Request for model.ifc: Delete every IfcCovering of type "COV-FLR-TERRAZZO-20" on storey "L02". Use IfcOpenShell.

First a look at what the model holds.

```python
import ifcopenshell
import ifcopenshell.util.element

model = ifcopenshell.open("model.ifc")
print(model.schema)
storey = next(s for s in model.by_type("IfcBuildingStorey") if s.Name == "L02")
coverings = [e for e in ifcopenshell.util.element.get_decomposition(storey) if e.is_a("IfcCovering")]
seen = {}
for e in coverings:
    element_type = ifcopenshell.util.element.get_type(e)
    name = element_type.Name if element_type not in (None, e) else None
    seen[name] = seen.get(name, 0) + 1
for name, count in sorted(seen.items(), key=str):
    print(count, "x", name)
```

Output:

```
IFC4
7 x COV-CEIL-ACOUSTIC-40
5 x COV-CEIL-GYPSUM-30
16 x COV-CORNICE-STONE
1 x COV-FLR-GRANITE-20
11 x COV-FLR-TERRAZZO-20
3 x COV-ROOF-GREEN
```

```python
import ifcopenshell
import ifcopenshell.api.root
import ifcopenshell.util.element

model = ifcopenshell.open("model.ifc")

storey = next(s for s in model.by_type("IfcBuildingStorey") if s.Name == "L02")
coverings = [e for e in ifcopenshell.util.element.get_decomposition(storey) if e.is_a("IfcCovering")]
targets = [e for e in coverings if (t := ifcopenshell.util.element.get_type(e)) not in (None, e) and t.Name == "COV-FLR-TERRAZZO-20"]

for e in targets:
    ifcopenshell.api.root.remove_product(model, product=e)
print(len(targets), "removed")

model.write("model-out.ifc")
```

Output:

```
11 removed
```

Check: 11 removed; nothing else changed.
